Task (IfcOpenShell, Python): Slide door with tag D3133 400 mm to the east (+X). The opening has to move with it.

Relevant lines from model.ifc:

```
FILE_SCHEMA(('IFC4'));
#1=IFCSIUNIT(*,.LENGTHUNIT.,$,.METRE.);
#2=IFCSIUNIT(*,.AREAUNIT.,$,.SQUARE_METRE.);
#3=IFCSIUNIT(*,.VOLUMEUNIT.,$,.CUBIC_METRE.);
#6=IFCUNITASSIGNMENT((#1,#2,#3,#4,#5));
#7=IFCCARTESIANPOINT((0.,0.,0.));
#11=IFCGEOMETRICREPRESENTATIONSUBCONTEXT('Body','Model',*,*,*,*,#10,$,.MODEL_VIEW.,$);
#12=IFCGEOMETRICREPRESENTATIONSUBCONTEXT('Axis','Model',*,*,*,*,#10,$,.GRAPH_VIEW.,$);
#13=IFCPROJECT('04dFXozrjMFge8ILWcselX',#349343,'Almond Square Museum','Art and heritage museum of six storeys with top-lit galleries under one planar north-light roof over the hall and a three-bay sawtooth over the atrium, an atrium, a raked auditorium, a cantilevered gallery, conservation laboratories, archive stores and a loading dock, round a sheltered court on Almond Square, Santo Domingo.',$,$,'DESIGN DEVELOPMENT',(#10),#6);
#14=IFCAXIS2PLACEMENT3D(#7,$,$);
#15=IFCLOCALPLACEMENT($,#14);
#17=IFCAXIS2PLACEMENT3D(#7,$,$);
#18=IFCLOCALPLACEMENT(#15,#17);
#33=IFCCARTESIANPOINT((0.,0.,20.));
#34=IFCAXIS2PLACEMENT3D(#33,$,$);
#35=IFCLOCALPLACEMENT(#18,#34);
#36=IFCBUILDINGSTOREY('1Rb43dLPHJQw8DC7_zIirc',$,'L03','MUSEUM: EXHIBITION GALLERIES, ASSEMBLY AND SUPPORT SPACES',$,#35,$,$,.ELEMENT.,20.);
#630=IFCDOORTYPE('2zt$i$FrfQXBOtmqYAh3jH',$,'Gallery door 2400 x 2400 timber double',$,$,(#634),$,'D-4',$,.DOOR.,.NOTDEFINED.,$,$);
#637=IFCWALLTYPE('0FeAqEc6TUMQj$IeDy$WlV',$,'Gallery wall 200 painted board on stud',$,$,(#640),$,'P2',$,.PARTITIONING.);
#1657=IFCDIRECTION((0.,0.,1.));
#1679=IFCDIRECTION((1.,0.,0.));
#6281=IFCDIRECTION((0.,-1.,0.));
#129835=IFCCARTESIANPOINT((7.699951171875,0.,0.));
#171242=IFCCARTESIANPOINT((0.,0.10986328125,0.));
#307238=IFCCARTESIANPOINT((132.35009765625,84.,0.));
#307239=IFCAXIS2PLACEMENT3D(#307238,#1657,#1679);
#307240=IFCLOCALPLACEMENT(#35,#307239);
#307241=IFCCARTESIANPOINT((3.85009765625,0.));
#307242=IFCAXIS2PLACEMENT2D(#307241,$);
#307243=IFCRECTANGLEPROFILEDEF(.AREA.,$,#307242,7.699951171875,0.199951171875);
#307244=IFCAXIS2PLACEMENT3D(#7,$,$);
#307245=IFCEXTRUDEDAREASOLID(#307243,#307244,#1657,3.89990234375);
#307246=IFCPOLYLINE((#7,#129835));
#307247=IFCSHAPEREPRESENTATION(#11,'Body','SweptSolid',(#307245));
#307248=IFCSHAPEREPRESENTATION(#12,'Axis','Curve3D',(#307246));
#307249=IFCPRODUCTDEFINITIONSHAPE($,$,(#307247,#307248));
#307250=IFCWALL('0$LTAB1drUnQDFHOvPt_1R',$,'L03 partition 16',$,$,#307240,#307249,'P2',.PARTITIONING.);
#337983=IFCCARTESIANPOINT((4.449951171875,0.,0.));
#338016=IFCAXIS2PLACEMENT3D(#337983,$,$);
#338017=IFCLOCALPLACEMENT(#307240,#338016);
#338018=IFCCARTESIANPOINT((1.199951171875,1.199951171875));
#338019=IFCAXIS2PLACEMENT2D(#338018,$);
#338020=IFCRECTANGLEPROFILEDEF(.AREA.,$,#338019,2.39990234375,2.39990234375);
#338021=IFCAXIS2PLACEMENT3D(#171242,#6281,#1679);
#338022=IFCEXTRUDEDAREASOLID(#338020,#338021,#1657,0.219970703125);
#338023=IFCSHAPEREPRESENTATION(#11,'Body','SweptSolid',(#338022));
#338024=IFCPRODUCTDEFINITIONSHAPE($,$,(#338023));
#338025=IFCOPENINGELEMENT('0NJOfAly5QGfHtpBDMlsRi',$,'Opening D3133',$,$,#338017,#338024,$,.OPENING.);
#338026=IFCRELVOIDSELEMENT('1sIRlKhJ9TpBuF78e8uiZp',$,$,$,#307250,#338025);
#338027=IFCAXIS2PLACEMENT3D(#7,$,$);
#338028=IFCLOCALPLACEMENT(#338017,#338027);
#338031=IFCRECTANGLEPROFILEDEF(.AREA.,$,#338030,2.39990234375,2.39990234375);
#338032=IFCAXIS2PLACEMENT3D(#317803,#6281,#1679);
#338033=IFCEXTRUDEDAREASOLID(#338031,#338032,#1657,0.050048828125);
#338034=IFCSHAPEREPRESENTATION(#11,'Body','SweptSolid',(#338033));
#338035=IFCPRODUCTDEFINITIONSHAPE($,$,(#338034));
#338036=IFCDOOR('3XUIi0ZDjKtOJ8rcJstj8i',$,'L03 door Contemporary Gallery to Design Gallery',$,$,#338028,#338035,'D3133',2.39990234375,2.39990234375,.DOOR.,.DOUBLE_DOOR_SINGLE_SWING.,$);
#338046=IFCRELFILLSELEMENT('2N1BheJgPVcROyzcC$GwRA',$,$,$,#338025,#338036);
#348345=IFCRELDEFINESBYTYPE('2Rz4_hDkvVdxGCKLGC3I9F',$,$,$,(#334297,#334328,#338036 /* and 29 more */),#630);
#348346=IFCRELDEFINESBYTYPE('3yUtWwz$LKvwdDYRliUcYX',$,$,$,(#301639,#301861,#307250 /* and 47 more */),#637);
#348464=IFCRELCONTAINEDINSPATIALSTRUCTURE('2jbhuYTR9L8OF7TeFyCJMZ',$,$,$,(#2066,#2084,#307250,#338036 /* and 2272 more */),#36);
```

```python
import ifcopenshell
import ifcopenshell.api.geometry
import ifcopenshell.util.placement
import ifcopenshell.util.unit

model = ifcopenshell.open("model.ifc")
unit_scale = ifcopenshell.util.unit.calculate_unit_scale(model)

door = model.by_id(338036)
opening = door.FillsVoids[0].RelatingOpeningElement
wall = opening.VoidsElements[0].RelatingBuildingElement

wall_matrix = ifcopenshell.util.placement.get_local_placement(wall.ObjectPlacement)
shift = wall_matrix[:3, 0] * 0.4 / unit_scale
before = ifcopenshell.util.placement.get_local_placement(door.ObjectPlacement)[:3, 3].copy()

# The door is placed relative to its opening, so it follows when the opening moves.
matrix = ifcopenshell.util.placement.get_local_placement(opening.ObjectPlacement)
matrix[:3, 3] += shift
ifcopenshell.api.geometry.edit_object_placement(
    model, product=opening, matrix=matrix, is_si=False, should_transform_children=True
)

after = ifcopenshell.util.placement.get_local_placement(door.ObjectPlacement)[:3, 3]
print("door moved by", (after - before).round(3) + 0.0)

model.write("model_updated.ifc")
```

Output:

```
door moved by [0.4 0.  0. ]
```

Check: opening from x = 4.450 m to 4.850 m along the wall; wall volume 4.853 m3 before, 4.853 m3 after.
